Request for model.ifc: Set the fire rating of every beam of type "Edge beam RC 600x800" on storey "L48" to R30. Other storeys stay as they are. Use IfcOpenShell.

First a look at what the model holds.

```python
import ifcopenshell
import ifcopenshell.util.element

model = ifcopenshell.open("model.ifc")
print(model.schema)
storey = next(s for s in model.by_type("IfcBuildingStorey") if s.Name == "L48")
beams = [e for e in ifcopenshell.util.element.get_decomposition(storey) if e.is_a("IfcBeam")]
seen = {}
for e in beams:
    element_type = ifcopenshell.util.element.get_type(e)
    key = (element_type.Name if element_type != e and element_type else None, ifcopenshell.util.element.get_pset(e, "Pset_BeamCommon", "FireRating"))
    seen[key] = seen.get(key, 0) + 1
for (name, value), count in sorted(seen.items(), key=str):
    print(count, "x", name, "|", value)
```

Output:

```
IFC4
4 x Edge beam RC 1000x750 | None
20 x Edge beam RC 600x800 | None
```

```python
import ifcopenshell
import ifcopenshell.api.pset
import ifcopenshell.util.element

model = ifcopenshell.open("model.ifc")

storey = next(s for s in model.by_type("IfcBuildingStorey") if s.Name == "L48")
beams = [e for e in ifcopenshell.util.element.get_decomposition(storey) if e.is_a("IfcBeam")]

count = 0
for e in beams:
    element_type = ifcopenshell.util.element.get_type(e)
    if element_type in (None, e) or element_type.Name != "Edge beam RC 600x800":
        continue
    found = ifcopenshell.util.element.get_pset(e, "Pset_BeamCommon", should_inherit=False)
    if found:
        pset = model.by_id(found["id"])
        if len(ifcopenshell.util.element.get_elements_by_pset(pset)) > 1:
            pset = ifcopenshell.api.pset.unshare_pset(model, products=[e], pset=pset)[0]
    else:
        pset = ifcopenshell.api.pset.add_pset(model, product=e, name="Pset_BeamCommon")
    ifcopenshell.api.pset.edit_pset(model, pset=pset, properties={"FireRating": "R30"})
    count += 1

print(count, "beams updated")

model.write("model-out.ifc")
```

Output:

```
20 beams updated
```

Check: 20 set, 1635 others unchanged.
